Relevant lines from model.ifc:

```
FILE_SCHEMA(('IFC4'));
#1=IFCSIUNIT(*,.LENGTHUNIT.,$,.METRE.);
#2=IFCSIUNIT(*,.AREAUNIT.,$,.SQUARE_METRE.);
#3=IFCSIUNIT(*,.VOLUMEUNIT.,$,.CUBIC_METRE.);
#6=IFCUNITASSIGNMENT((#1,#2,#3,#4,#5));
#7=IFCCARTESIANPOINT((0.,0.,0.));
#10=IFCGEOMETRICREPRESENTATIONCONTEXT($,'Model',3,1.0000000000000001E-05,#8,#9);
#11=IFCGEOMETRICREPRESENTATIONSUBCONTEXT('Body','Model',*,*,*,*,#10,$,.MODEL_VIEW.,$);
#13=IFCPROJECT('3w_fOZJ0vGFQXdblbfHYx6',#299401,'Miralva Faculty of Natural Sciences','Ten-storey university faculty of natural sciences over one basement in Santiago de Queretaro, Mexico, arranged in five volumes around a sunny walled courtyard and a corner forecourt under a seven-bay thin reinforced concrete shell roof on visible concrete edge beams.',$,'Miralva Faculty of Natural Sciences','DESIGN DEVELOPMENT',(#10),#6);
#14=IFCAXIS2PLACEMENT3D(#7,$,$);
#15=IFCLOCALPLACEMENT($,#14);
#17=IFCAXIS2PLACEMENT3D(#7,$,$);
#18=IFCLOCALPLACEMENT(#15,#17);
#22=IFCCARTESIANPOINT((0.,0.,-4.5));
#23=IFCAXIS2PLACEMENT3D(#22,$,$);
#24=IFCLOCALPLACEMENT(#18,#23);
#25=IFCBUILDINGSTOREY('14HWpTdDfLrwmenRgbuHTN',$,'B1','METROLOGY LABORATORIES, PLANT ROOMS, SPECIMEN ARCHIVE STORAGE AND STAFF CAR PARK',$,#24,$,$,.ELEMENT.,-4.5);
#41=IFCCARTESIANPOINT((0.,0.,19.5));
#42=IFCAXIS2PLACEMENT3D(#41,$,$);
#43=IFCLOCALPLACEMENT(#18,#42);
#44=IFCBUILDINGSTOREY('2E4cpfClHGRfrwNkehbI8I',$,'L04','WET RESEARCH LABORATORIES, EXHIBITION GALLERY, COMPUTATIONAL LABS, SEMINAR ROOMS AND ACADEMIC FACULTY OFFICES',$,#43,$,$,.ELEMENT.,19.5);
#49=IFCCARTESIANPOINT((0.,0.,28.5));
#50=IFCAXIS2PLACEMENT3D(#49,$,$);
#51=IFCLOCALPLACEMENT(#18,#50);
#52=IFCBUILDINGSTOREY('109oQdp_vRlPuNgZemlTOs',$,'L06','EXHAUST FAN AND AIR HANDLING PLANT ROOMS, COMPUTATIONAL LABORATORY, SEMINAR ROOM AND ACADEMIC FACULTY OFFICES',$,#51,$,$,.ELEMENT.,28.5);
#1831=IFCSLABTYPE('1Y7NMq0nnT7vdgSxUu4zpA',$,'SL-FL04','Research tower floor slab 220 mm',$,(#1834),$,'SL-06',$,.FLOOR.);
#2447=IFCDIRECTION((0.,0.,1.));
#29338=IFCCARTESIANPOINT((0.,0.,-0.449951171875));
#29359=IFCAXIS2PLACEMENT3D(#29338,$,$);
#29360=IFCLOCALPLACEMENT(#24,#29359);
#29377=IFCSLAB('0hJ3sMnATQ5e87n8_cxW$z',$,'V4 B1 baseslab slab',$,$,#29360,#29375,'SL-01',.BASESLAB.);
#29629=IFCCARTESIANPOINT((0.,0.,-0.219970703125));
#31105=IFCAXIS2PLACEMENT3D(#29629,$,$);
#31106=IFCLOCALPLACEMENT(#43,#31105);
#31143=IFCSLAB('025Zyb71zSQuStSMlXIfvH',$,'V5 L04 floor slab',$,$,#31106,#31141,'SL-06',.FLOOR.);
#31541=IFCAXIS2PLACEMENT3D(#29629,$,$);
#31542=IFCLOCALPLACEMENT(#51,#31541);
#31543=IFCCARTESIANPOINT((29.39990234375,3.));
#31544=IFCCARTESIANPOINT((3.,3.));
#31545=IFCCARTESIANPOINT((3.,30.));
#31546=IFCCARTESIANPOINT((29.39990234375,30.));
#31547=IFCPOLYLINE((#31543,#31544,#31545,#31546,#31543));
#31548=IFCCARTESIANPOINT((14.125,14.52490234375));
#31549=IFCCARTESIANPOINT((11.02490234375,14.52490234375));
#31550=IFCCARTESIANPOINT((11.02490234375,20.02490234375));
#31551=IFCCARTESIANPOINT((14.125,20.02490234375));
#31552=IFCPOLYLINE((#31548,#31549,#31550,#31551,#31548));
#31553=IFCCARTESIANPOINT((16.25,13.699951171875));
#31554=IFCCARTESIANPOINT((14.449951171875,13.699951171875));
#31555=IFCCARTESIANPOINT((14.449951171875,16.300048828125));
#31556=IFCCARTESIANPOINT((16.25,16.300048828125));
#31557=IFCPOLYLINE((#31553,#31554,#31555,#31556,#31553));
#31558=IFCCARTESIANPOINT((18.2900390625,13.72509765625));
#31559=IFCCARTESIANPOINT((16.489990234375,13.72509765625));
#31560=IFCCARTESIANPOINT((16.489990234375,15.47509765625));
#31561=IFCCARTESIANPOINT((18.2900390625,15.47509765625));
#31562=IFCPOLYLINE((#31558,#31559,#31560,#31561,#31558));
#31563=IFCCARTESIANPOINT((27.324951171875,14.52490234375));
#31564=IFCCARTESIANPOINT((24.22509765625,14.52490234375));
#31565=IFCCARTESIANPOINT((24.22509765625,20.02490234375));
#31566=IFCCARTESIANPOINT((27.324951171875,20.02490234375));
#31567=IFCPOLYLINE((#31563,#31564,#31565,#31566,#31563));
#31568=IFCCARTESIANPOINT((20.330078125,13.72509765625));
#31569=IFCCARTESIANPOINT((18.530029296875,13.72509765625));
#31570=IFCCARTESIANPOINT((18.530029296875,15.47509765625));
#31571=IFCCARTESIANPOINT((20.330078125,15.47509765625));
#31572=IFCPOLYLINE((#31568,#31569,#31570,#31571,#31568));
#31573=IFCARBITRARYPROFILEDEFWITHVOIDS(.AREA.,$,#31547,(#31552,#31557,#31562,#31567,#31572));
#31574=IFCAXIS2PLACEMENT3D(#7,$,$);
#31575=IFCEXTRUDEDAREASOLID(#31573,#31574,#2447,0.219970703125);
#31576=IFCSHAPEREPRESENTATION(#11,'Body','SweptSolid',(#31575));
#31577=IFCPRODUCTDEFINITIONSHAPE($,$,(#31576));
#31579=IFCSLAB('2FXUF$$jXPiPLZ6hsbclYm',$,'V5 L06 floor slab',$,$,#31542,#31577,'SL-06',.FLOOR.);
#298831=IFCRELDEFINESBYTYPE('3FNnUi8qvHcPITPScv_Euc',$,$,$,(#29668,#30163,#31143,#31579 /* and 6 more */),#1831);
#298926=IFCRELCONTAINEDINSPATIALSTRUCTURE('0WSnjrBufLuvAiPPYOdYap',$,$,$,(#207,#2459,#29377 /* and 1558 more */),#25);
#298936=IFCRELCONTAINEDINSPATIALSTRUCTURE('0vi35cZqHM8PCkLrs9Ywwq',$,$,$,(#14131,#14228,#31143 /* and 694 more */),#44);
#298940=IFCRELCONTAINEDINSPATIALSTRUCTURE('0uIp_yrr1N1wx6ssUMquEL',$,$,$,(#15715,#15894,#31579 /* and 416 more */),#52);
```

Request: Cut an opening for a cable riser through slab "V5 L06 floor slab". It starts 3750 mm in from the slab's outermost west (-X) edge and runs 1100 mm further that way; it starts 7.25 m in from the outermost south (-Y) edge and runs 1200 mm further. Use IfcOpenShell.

```python
import numpy as np
import ifcopenshell
import ifcopenshell.api.feature
import ifcopenshell.api.geometry
import ifcopenshell.api.root
import ifcopenshell.geom
import ifcopenshell.util.placement
import ifcopenshell.util.representation
import ifcopenshell.util.shape
import ifcopenshell.util.unit

model = ifcopenshell.open("model.ifc")
unit_scale = ifcopenshell.util.unit.calculate_unit_scale(model)
settings = ifcopenshell.geom.settings()


def volume(element):
    """Net volume in cubic metres, openings subtracted."""
    shape = ifcopenshell.geom.create_shape(settings, element)
    return ifcopenshell.util.shape.get_volume(shape.geometry)


slab = model.by_guid("2FXUF$$jXPiPLZ6hsbclYm")
before = volume(slab)

# Extent in the slab's own axes, in metres. The edges named are its -X and -Y sides.
slab_shape = ifcopenshell.geom.create_shape(settings, slab)
vertices = ifcopenshell.util.shape.get_vertices(slab_shape.geometry)
x_min, y_min, bottom = vertices.min(axis=0)
top = vertices[:, 2].max()

opening = ifcopenshell.api.root.create_entity(model, ifc_class="IfcOpeningElement", name="Cable riser opening", predefined_type="OPENING")
context = ifcopenshell.util.representation.get_context(model, "Model", "Body", "MODEL_VIEW")
width, depth = 1.1, 1.2
outline = [(0.0, 0.0), (width, 0.0), (width, depth), (0.0, depth), (0.0, 0.0)]
# Overshoot both faces by 50 mm so the cut is clean.
shape = ifcopenshell.api.geometry.add_slab_representation(
    model, context=context, depth=top - bottom + 0.1, polyline=outline
)
ifcopenshell.api.geometry.assign_representation(model, product=opening, representation=shape)

matrix = ifcopenshell.util.placement.get_local_placement(slab.ObjectPlacement)
matrix[:, 3] = matrix @ np.append(np.array([x_min + 3.75, y_min + 7.25, bottom - 0.05]) / unit_scale, 1.0)
ifcopenshell.api.geometry.edit_object_placement(model, product=opening, matrix=matrix, is_si=False)
ifcopenshell.api.feature.add_feature(model, feature=opening, element=slab)

after = volume(slab)

print(f"slab volume {before:.3f} -> {after:.3f} m3")

model.write("model-out.ifc")
```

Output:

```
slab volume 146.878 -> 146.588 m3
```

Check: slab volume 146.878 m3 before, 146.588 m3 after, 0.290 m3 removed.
